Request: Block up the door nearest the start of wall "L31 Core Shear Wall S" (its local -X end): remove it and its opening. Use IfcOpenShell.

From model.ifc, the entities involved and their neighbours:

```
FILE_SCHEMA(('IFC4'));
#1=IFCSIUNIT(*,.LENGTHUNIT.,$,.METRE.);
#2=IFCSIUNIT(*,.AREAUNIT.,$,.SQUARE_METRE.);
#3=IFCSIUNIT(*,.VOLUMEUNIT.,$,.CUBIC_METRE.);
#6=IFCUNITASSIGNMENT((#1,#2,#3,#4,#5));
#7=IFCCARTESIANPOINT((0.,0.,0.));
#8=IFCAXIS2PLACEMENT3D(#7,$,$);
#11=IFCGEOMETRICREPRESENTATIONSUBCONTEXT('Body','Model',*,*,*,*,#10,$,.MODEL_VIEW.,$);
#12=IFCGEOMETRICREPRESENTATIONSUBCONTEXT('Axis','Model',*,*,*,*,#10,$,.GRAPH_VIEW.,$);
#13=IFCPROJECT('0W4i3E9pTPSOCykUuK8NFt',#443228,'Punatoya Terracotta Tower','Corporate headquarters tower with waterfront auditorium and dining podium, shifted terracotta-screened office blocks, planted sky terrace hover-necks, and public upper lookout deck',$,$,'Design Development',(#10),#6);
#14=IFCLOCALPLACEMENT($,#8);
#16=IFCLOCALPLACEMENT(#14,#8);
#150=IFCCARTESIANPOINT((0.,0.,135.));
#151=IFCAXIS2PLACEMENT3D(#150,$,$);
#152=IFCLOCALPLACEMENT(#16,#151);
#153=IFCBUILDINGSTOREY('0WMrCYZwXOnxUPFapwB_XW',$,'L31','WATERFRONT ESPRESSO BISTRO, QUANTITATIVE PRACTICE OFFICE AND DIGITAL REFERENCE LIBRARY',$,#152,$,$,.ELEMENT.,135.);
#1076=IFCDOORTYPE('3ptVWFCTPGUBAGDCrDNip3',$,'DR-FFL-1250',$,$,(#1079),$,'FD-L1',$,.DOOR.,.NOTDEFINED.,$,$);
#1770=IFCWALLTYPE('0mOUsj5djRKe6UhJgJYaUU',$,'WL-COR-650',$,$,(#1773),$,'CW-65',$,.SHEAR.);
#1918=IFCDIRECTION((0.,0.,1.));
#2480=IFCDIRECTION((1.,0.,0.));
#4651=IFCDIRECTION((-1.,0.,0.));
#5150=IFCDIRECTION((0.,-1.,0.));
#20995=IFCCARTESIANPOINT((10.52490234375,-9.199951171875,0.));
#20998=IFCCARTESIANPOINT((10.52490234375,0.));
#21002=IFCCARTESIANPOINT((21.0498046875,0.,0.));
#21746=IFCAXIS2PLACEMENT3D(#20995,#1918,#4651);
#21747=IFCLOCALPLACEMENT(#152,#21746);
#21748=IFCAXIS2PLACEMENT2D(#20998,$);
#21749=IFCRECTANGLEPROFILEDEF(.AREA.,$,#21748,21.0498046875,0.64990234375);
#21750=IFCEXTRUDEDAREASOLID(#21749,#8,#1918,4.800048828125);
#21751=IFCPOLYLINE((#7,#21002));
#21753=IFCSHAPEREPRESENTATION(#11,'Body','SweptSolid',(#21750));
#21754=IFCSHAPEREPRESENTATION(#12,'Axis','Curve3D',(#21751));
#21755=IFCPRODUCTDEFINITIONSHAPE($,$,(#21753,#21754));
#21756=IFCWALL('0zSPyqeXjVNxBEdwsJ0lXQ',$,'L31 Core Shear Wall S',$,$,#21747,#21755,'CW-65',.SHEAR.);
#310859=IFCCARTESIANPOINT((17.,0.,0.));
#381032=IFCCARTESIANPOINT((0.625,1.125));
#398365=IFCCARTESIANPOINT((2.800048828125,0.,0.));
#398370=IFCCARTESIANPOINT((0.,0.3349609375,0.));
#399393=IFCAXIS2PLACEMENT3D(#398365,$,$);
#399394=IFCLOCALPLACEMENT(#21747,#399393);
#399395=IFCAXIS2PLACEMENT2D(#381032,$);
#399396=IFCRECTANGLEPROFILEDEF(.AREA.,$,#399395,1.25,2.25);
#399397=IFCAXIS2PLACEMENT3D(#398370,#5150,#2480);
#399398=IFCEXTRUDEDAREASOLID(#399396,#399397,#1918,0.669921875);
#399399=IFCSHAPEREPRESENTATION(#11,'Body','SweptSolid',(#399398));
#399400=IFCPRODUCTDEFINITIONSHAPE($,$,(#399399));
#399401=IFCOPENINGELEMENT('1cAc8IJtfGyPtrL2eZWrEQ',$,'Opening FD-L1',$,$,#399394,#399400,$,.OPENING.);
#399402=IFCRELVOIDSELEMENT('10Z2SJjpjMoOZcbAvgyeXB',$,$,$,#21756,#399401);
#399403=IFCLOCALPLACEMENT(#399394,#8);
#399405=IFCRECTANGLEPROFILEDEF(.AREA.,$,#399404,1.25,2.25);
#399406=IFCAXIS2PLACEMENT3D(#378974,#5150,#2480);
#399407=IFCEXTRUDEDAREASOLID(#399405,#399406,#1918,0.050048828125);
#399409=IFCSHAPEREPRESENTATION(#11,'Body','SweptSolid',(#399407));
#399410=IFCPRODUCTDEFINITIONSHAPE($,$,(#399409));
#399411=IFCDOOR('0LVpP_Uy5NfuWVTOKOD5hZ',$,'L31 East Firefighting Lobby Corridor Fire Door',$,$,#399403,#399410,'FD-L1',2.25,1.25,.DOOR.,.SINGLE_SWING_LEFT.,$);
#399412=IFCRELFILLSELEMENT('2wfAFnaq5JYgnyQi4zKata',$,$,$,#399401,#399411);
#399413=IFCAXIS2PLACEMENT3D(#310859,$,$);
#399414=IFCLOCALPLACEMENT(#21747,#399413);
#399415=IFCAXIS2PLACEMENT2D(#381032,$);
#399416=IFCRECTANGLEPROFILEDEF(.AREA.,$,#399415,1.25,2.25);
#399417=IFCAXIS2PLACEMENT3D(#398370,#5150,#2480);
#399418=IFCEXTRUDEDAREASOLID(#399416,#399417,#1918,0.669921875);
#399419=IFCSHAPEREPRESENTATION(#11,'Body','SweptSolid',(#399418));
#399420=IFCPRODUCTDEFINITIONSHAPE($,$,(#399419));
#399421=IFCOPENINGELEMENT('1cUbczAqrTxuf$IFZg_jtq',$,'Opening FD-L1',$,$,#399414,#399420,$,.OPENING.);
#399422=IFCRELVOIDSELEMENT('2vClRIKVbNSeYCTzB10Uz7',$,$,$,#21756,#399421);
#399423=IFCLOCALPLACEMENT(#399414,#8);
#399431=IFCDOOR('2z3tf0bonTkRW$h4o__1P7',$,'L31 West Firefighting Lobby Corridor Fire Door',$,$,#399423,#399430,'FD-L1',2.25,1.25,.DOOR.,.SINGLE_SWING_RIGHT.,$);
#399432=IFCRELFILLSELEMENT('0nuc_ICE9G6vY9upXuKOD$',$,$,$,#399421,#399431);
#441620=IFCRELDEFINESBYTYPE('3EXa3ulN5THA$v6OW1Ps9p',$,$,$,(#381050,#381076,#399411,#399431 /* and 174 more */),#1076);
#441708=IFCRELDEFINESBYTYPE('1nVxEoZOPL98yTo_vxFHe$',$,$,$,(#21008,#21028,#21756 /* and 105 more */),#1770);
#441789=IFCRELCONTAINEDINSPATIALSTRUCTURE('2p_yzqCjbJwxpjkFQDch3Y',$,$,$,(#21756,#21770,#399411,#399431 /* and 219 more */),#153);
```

```python
import ifcopenshell
import ifcopenshell.api.feature
import ifcopenshell.api.root
import ifcopenshell.geom
import ifcopenshell.util.shape

model = ifcopenshell.open("model.ifc")
settings = ifcopenshell.geom.settings()


def volume(element):
    """Net volume in cubic metres, openings subtracted."""
    shape = ifcopenshell.geom.create_shape(settings, element)
    return ifcopenshell.util.shape.get_volume(shape.geometry)


door = model.by_guid("0LVpP_Uy5NfuWVTOKOD5hZ")
opening = door.FillsVoids[0].RelatingOpeningElement
wall = opening.VoidsElements[0].RelatingBuildingElement
before = volume(wall)

ifcopenshell.api.root.remove_product(model, product=door)
ifcopenshell.api.feature.remove_feature(model, feature=opening)

after = volume(wall)

print(f"wall volume {before:.3f} -> {after:.3f} m3")

model.write("model_rev.ifc")
```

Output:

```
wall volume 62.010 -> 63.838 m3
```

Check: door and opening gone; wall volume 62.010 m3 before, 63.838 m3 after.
